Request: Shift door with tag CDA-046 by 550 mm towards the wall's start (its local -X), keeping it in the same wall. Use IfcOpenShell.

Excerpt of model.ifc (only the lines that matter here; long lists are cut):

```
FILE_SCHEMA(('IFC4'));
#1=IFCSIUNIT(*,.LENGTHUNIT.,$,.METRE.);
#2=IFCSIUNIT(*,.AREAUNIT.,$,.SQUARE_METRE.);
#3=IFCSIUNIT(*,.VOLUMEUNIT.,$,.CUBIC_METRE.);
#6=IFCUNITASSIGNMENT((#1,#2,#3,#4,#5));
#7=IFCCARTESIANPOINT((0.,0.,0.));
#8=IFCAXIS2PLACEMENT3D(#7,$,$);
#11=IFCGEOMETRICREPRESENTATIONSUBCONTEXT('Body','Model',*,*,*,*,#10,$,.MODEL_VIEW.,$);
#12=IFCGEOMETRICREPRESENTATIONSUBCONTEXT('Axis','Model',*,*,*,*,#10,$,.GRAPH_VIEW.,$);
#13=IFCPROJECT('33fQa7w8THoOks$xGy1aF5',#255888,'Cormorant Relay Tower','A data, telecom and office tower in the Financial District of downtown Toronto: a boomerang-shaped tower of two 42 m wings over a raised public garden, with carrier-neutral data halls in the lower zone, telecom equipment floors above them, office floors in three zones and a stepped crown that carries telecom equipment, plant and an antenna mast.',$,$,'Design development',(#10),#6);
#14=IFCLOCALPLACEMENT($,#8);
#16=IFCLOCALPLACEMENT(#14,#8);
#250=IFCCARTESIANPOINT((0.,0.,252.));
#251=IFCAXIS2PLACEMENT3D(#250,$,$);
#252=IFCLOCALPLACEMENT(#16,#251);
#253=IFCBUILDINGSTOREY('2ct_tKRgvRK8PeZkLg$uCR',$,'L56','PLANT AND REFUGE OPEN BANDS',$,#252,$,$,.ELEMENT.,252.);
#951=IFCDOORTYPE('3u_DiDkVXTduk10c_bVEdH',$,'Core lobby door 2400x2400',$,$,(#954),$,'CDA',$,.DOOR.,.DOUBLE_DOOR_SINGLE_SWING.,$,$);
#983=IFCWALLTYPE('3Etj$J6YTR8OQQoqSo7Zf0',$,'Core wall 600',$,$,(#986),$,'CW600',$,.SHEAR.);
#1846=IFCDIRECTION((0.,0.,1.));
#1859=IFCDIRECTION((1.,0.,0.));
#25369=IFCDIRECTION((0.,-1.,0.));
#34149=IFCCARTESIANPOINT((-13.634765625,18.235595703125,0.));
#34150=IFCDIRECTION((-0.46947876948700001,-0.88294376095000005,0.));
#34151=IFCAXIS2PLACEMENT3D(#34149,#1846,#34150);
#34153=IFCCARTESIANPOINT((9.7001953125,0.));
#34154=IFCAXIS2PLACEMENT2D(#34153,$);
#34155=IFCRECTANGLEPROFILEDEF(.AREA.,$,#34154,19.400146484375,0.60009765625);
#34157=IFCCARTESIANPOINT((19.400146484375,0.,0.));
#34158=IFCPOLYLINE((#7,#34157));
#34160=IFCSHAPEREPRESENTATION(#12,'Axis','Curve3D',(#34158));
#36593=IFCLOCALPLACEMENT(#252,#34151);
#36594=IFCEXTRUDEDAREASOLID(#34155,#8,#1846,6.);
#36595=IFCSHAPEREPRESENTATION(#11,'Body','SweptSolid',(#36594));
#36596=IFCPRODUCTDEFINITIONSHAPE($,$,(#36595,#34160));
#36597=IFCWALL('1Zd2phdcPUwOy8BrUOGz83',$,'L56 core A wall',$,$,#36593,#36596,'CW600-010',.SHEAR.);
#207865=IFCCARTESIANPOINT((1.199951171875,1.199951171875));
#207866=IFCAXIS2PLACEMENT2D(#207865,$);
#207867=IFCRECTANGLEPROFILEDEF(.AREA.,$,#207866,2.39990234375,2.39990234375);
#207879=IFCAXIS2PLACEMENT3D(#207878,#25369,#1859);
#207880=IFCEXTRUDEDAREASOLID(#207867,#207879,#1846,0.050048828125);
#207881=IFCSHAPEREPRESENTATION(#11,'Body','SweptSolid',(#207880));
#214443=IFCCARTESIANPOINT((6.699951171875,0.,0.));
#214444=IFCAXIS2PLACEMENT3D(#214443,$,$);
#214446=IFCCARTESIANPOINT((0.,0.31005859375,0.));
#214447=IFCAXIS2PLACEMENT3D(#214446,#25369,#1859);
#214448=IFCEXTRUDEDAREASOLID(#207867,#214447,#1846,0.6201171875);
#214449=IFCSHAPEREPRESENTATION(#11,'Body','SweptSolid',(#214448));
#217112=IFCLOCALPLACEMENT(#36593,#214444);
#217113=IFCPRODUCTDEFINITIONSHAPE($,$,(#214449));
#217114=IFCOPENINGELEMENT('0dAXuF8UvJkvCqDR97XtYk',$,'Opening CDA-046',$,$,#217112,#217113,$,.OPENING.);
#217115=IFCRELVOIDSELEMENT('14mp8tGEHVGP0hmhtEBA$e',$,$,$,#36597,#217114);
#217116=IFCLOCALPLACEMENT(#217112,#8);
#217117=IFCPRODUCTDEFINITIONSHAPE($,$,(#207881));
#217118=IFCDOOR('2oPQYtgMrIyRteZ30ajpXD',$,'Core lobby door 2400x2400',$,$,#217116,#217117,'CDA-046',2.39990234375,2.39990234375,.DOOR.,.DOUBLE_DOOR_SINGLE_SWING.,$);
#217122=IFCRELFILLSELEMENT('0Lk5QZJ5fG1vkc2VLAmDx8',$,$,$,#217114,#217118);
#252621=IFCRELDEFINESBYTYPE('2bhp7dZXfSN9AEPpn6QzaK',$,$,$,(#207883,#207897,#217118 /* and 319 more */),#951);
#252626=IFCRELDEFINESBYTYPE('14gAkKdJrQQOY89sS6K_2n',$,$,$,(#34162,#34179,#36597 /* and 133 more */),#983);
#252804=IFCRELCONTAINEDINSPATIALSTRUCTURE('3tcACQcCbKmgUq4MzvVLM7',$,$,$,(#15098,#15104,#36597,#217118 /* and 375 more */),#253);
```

```python
import ifcopenshell
import ifcopenshell.api.geometry
import ifcopenshell.util.placement
import ifcopenshell.util.unit

model = ifcopenshell.open("model.ifc")
unit_scale = ifcopenshell.util.unit.calculate_unit_scale(model)

door = model.by_guid("2oPQYtgMrIyRteZ30ajpXD")
opening = door.FillsVoids[0].RelatingOpeningElement
wall = opening.VoidsElements[0].RelatingBuildingElement

wall_matrix = ifcopenshell.util.placement.get_local_placement(wall.ObjectPlacement)
shift = wall_matrix[:3, 0] * -0.55 / unit_scale
before = ifcopenshell.util.placement.get_local_placement(door.ObjectPlacement)[:3, 3].copy()

# The door is placed relative to its opening, so it follows when the opening moves.
matrix = ifcopenshell.util.placement.get_local_placement(opening.ObjectPlacement)
matrix[:3, 3] += shift
ifcopenshell.api.geometry.edit_object_placement(
    model, product=opening, matrix=matrix, is_si=False, should_transform_children=True
)

after = ifcopenshell.util.placement.get_local_placement(door.ObjectPlacement)[:3, 3]
print("door moved by", (after - before).round(3) + 0.0)

model.write("model_edited.ifc")
```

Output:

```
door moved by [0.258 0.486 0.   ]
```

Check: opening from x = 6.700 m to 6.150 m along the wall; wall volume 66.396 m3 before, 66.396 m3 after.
